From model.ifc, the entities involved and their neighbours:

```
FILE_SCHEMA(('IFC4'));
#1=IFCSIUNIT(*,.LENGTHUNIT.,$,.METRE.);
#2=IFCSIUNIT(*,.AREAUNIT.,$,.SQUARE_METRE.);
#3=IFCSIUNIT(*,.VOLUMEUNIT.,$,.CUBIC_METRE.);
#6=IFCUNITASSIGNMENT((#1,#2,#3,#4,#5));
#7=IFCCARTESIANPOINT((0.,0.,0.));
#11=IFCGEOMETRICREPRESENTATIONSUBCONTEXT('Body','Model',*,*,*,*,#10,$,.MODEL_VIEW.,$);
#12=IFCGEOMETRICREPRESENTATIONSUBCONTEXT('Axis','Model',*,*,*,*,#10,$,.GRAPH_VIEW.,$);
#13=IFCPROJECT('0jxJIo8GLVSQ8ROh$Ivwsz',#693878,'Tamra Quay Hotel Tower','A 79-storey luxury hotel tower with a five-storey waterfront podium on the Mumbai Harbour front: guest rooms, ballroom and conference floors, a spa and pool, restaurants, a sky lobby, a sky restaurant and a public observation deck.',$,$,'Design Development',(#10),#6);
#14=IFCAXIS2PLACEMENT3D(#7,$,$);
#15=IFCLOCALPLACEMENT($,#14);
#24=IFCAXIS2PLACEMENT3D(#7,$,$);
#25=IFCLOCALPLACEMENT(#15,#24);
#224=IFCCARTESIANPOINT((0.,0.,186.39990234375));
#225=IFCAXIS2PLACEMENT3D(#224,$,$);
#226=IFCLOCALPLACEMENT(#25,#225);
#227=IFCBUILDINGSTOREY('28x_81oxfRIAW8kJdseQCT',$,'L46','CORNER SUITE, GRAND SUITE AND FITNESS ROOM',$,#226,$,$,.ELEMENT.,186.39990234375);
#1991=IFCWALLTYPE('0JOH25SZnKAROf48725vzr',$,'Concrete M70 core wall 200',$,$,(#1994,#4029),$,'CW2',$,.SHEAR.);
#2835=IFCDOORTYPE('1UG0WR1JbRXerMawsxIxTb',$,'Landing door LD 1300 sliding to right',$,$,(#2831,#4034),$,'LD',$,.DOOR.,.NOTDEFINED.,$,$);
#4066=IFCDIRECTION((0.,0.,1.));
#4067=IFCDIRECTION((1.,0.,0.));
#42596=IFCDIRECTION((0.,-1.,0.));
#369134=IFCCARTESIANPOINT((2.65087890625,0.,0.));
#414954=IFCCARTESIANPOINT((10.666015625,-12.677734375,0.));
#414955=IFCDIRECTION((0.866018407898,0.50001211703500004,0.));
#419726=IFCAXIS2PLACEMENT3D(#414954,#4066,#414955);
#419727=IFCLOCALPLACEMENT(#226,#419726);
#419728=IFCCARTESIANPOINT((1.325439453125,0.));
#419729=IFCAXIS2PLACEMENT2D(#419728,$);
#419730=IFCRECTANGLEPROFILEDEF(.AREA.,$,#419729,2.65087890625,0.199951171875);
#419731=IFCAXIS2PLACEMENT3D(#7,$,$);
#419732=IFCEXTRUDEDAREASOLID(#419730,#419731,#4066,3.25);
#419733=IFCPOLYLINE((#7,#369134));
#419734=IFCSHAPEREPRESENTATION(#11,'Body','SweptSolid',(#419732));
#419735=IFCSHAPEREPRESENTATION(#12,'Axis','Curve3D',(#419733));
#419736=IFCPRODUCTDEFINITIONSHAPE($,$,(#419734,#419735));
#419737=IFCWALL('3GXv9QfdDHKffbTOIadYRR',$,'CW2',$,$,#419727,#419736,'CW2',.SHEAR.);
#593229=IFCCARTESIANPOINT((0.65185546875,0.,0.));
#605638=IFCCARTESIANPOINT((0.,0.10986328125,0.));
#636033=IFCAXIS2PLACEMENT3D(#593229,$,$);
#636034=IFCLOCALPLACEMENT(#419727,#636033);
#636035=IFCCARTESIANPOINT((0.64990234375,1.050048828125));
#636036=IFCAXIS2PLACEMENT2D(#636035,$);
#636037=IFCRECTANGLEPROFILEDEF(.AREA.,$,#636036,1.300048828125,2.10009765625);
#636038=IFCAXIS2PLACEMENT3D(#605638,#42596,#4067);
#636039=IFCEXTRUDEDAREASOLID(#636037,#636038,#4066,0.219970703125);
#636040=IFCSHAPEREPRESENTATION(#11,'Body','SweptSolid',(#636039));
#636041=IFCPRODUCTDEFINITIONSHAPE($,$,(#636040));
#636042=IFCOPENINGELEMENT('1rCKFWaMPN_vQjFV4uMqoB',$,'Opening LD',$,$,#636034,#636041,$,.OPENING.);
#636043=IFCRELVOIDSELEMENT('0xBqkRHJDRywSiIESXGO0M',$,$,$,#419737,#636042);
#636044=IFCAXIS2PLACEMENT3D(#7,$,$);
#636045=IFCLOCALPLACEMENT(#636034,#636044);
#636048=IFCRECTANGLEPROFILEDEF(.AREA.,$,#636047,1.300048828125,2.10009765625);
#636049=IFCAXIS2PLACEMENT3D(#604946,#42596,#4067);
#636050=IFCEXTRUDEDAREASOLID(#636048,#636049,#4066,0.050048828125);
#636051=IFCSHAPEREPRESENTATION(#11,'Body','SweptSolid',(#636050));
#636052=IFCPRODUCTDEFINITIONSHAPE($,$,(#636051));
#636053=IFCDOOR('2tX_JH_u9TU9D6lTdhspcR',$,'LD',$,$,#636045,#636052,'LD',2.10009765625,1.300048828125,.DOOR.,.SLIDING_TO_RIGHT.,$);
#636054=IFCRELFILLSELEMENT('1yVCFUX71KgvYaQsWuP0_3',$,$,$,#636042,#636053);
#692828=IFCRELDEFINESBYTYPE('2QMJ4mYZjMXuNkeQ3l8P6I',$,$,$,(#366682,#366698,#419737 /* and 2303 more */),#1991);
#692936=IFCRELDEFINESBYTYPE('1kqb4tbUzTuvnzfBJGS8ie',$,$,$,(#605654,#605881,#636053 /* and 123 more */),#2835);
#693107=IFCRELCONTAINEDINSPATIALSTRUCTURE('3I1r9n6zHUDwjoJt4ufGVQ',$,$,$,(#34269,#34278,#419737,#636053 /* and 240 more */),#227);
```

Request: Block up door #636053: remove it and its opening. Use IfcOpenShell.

```python
import ifcopenshell
import ifcopenshell.api.feature
import ifcopenshell.api.root
import ifcopenshell.geom
import ifcopenshell.util.shape

model = ifcopenshell.open("model.ifc")
settings = ifcopenshell.geom.settings()


def volume(element):
    """Net volume in cubic metres, openings subtracted."""
    shape = ifcopenshell.geom.create_shape(settings, element)
    return ifcopenshell.util.shape.get_volume(shape.geometry)


door = model.by_id(636053)
opening = door.FillsVoids[0].RelatingOpeningElement
wall = opening.VoidsElements[0].RelatingBuildingElement
before = volume(wall)

ifcopenshell.api.root.remove_product(model, product=door)
ifcopenshell.api.feature.remove_feature(model, feature=opening)

after = volume(wall)

print(f"wall volume {before:.3f} -> {after:.3f} m3")

model.write("model_rev.ifc")
```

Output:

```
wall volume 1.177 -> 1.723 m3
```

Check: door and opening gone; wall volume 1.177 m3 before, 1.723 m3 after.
